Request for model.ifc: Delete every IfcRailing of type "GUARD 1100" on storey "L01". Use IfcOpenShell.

First a look at what the model holds.

```python
import ifcopenshell
import ifcopenshell.util.element

model = ifcopenshell.open("model.ifc")
print(model.schema)
storey = next(s for s in model.by_type("IfcBuildingStorey") if s.Name == "L01")
railings = [e for e in ifcopenshell.util.element.get_decomposition(storey) if e.is_a("IfcRailing")]
seen = {}
for e in railings:
    element_type = ifcopenshell.util.element.get_type(e)
    name = element_type.Name if element_type not in (None, e) else None
    seen[name] = seen.get(name, 0) + 1
for name, count in sorted(seen.items(), key=str):
    print(count, "x", name)
```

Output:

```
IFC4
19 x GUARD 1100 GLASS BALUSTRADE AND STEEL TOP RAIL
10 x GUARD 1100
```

```python
import ifcopenshell
import ifcopenshell.api.root
import ifcopenshell.util.element

model = ifcopenshell.open("model.ifc")

storey = next(s for s in model.by_type("IfcBuildingStorey") if s.Name == "L01")
railings = [e for e in ifcopenshell.util.element.get_decomposition(storey) if e.is_a("IfcRailing")]
targets = [e for e in railings if (t := ifcopenshell.util.element.get_type(e)) not in (None, e) and t.Name == "GUARD 1100"]

for e in targets:
    ifcopenshell.api.root.remove_product(model, product=e)
print(len(targets), "removed")

model.write("model_edited.ifc")
```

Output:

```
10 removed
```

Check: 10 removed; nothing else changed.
